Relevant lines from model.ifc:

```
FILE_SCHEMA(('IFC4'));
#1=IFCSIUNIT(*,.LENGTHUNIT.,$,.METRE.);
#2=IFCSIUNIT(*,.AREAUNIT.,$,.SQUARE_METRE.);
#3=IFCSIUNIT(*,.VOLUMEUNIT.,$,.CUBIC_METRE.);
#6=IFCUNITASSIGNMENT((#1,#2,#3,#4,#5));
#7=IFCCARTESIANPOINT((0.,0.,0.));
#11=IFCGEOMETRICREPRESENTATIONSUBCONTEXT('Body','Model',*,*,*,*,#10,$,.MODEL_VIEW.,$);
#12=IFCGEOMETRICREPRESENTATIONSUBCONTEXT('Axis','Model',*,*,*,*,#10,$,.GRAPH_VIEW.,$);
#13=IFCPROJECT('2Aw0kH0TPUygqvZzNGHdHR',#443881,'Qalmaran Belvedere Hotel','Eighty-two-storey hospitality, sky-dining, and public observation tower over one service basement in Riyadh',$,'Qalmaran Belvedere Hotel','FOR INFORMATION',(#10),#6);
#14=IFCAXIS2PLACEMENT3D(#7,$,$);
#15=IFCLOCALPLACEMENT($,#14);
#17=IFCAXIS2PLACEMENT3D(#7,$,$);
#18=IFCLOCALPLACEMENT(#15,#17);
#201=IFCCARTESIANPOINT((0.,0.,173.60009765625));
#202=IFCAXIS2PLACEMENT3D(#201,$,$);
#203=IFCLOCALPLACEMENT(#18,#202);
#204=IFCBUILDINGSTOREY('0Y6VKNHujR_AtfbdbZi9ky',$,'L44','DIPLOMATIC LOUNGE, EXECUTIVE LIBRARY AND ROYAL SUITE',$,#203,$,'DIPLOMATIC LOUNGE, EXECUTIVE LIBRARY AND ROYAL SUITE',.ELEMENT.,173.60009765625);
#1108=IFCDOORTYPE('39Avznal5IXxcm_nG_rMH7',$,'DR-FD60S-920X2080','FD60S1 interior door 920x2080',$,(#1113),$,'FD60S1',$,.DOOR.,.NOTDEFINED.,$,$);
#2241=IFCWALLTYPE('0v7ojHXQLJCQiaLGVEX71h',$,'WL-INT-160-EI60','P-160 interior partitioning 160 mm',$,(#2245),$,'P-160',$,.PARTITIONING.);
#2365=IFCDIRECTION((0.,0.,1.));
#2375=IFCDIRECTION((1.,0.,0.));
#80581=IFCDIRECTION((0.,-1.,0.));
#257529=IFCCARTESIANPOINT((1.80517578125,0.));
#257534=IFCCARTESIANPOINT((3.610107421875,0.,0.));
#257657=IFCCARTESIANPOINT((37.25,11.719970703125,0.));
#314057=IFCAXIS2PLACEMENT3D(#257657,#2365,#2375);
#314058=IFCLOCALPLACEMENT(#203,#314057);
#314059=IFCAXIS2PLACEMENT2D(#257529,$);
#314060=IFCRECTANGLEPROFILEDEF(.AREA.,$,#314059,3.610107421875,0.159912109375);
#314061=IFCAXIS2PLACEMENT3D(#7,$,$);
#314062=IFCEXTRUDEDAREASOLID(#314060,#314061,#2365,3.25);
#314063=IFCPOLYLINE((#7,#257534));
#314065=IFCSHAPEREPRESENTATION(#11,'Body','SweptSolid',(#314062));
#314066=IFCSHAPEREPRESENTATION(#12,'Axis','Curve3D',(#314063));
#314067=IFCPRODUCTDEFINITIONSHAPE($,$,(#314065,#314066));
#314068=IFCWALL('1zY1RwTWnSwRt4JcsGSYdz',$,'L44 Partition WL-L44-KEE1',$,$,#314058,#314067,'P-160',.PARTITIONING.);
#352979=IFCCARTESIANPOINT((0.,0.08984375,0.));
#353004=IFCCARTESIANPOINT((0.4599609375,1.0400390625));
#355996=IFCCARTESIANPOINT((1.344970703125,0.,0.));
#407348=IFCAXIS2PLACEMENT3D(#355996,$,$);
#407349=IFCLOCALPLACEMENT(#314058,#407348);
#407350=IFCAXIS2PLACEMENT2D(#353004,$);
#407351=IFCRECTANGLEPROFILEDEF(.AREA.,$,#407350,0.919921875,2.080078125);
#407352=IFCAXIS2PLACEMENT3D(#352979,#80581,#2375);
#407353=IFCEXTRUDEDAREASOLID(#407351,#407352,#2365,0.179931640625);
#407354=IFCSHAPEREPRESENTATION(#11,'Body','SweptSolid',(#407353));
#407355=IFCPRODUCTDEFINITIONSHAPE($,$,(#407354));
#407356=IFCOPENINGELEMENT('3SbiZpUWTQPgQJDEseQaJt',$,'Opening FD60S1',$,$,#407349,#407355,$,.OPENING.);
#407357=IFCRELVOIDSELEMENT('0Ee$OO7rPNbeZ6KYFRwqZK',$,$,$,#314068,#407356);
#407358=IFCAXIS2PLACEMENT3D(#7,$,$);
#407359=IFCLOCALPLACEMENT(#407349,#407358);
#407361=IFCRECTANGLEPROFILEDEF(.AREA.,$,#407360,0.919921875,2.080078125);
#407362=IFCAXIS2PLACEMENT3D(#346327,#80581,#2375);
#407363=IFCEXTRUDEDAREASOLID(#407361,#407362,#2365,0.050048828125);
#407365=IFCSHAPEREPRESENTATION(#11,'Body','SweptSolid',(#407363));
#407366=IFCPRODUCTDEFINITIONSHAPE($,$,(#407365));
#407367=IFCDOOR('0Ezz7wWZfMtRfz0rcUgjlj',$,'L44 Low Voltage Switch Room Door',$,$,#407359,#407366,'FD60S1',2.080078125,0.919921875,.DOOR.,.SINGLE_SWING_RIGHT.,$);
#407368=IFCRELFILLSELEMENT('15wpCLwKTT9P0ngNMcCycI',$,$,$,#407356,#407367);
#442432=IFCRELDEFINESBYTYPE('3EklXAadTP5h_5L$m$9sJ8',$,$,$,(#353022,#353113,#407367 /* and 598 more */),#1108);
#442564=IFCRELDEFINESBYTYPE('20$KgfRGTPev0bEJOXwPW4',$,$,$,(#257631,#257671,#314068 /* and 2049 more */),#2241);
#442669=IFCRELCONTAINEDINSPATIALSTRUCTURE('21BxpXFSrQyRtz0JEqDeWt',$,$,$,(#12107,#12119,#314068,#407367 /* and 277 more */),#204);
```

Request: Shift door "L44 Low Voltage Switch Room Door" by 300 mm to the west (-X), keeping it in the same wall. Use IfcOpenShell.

```python
import ifcopenshell
import ifcopenshell.api.geometry
import ifcopenshell.util.placement

model = ifcopenshell.open("model.ifc")

door = model.by_guid("0Ezz7wWZfMtRfz0rcUgjlj")
opening = door.FillsVoids[0].RelatingOpeningElement
wall = opening.VoidsElements[0].RelatingBuildingElement

wall_matrix = ifcopenshell.util.placement.get_local_placement(wall.ObjectPlacement)
shift = wall_matrix[:3, 0] * -0.3
before = ifcopenshell.util.placement.get_local_placement(door.ObjectPlacement)[:3, 3].copy()

# The door is placed relative to its opening, so it follows when the opening moves.
matrix = ifcopenshell.util.placement.get_local_placement(opening.ObjectPlacement)
matrix[:3, 3] += shift
ifcopenshell.api.geometry.edit_object_placement(
    model, product=opening, matrix=matrix, is_si=False, should_transform_children=True
)

after = ifcopenshell.util.placement.get_local_placement(door.ObjectPlacement)[:3, 3]
print("door moved by", (after - before).round(3) + 0.0)

model.write("model_updated.ifc")
```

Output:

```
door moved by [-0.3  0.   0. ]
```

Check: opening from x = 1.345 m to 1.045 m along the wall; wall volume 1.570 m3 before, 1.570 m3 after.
